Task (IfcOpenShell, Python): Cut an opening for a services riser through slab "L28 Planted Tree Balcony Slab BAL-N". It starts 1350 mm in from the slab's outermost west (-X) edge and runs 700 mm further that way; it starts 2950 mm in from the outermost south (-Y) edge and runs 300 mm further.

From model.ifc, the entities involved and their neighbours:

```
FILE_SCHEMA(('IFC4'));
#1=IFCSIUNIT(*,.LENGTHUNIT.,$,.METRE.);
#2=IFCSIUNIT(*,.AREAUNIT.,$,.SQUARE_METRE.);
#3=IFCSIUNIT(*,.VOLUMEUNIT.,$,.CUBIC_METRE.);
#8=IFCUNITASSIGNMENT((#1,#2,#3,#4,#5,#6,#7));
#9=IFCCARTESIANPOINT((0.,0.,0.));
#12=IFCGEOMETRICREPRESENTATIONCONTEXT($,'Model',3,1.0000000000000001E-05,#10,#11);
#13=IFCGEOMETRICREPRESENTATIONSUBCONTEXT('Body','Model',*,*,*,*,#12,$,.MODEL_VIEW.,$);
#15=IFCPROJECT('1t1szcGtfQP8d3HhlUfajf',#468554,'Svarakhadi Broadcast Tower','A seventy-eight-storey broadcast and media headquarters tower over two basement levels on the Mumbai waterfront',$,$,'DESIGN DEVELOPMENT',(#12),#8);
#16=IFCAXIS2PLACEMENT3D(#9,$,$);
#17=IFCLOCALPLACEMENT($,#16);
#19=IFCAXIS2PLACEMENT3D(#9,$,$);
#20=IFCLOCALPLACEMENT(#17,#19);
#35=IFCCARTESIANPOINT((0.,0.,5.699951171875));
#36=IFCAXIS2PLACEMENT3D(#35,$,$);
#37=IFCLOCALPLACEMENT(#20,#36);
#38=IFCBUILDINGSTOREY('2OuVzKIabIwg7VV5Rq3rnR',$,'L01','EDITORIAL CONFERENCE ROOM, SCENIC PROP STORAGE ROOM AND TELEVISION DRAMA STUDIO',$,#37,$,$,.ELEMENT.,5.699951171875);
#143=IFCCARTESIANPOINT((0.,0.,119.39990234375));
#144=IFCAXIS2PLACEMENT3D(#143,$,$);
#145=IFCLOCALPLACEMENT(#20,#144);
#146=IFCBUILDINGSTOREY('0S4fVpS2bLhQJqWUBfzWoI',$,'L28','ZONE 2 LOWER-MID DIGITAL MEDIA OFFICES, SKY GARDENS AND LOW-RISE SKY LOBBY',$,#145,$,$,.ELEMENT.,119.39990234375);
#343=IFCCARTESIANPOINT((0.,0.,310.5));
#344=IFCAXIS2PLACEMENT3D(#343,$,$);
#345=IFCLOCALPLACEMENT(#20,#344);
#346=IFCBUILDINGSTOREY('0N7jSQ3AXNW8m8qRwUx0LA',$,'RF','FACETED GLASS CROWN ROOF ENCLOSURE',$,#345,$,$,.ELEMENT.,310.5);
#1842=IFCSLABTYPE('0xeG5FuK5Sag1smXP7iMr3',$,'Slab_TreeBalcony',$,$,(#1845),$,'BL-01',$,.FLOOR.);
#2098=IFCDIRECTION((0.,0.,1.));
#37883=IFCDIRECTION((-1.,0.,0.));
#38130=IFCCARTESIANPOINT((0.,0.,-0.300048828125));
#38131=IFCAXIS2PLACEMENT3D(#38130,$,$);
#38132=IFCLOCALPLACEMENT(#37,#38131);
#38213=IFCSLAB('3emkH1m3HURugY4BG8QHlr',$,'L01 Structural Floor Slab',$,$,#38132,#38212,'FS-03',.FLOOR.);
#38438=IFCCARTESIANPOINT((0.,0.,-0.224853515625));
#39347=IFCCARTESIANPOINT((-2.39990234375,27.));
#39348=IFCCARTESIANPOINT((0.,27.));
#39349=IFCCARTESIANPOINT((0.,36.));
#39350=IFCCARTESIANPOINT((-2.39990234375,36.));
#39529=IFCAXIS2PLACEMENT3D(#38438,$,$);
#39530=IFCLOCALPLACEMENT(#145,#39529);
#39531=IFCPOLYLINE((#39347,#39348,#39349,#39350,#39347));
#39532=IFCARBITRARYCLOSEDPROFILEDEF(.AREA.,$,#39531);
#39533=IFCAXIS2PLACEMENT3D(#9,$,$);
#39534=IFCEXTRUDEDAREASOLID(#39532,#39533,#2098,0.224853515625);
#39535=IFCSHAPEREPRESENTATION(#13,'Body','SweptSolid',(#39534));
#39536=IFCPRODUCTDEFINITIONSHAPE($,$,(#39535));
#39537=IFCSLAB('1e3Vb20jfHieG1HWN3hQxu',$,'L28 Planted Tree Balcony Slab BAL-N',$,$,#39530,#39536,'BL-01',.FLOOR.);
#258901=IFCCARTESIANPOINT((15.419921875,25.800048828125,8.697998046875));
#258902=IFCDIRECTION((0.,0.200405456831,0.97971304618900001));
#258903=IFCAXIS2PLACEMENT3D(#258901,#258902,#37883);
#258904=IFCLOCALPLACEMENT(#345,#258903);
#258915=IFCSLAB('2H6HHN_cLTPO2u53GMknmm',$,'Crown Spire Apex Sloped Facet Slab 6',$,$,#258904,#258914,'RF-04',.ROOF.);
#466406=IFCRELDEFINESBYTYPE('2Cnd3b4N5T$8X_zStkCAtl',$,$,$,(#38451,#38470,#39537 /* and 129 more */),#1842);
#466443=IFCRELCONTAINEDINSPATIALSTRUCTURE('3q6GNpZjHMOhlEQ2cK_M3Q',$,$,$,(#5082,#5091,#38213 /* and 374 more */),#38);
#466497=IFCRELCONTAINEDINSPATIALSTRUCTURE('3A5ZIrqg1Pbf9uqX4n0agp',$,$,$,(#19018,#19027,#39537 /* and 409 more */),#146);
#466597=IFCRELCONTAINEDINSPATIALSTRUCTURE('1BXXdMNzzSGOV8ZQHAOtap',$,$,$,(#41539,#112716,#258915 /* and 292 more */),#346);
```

```python
import numpy as np
import ifcopenshell
import ifcopenshell.api.feature
import ifcopenshell.api.geometry
import ifcopenshell.api.root
import ifcopenshell.geom
import ifcopenshell.util.placement
import ifcopenshell.util.representation
import ifcopenshell.util.shape
import ifcopenshell.util.unit

model = ifcopenshell.open("model.ifc")
unit_scale = ifcopenshell.util.unit.calculate_unit_scale(model)
settings = ifcopenshell.geom.settings()


def volume(element):
    """Net volume in cubic metres, openings subtracted."""
    shape = ifcopenshell.geom.create_shape(settings, element)
    return ifcopenshell.util.shape.get_volume(shape.geometry)


slab = model.by_guid("1e3Vb20jfHieG1HWN3hQxu")
before = volume(slab)

# Extent in the slab's own axes, in metres. The edges named are its -X and -Y sides.
slab_shape = ifcopenshell.geom.create_shape(settings, slab)
vertices = ifcopenshell.util.shape.get_vertices(slab_shape.geometry)
x_min, y_min, bottom = vertices.min(axis=0)
top = vertices[:, 2].max()

opening = ifcopenshell.api.root.create_entity(model, ifc_class="IfcOpeningElement", name="Services riser opening", predefined_type="OPENING")
context = ifcopenshell.util.representation.get_context(model, "Model", "Body", "MODEL_VIEW")
width, depth = 0.7, 0.3
outline = [(0.0, 0.0), (width, 0.0), (width, depth), (0.0, depth), (0.0, 0.0)]
# Overshoot both faces by 50 mm so the cut is clean.
shape = ifcopenshell.api.geometry.add_slab_representation(
    model, context=context, depth=top - bottom + 0.1, polyline=outline
)
ifcopenshell.api.geometry.assign_representation(model, product=opening, representation=shape)

matrix = ifcopenshell.util.placement.get_local_placement(slab.ObjectPlacement)
matrix[:, 3] = matrix @ np.append(np.array([x_min + 1.35, y_min + 2.95, bottom - 0.05]) / unit_scale, 1.0)
ifcopenshell.api.geometry.edit_object_placement(model, product=opening, matrix=matrix, is_si=False)
ifcopenshell.api.feature.add_feature(model, feature=opening, element=slab)

after = volume(slab)

print(f"slab volume {before:.3f} -> {after:.3f} m3")

model.write("model_rev.ifc")
```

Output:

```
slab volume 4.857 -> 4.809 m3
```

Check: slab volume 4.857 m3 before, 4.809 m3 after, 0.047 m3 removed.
